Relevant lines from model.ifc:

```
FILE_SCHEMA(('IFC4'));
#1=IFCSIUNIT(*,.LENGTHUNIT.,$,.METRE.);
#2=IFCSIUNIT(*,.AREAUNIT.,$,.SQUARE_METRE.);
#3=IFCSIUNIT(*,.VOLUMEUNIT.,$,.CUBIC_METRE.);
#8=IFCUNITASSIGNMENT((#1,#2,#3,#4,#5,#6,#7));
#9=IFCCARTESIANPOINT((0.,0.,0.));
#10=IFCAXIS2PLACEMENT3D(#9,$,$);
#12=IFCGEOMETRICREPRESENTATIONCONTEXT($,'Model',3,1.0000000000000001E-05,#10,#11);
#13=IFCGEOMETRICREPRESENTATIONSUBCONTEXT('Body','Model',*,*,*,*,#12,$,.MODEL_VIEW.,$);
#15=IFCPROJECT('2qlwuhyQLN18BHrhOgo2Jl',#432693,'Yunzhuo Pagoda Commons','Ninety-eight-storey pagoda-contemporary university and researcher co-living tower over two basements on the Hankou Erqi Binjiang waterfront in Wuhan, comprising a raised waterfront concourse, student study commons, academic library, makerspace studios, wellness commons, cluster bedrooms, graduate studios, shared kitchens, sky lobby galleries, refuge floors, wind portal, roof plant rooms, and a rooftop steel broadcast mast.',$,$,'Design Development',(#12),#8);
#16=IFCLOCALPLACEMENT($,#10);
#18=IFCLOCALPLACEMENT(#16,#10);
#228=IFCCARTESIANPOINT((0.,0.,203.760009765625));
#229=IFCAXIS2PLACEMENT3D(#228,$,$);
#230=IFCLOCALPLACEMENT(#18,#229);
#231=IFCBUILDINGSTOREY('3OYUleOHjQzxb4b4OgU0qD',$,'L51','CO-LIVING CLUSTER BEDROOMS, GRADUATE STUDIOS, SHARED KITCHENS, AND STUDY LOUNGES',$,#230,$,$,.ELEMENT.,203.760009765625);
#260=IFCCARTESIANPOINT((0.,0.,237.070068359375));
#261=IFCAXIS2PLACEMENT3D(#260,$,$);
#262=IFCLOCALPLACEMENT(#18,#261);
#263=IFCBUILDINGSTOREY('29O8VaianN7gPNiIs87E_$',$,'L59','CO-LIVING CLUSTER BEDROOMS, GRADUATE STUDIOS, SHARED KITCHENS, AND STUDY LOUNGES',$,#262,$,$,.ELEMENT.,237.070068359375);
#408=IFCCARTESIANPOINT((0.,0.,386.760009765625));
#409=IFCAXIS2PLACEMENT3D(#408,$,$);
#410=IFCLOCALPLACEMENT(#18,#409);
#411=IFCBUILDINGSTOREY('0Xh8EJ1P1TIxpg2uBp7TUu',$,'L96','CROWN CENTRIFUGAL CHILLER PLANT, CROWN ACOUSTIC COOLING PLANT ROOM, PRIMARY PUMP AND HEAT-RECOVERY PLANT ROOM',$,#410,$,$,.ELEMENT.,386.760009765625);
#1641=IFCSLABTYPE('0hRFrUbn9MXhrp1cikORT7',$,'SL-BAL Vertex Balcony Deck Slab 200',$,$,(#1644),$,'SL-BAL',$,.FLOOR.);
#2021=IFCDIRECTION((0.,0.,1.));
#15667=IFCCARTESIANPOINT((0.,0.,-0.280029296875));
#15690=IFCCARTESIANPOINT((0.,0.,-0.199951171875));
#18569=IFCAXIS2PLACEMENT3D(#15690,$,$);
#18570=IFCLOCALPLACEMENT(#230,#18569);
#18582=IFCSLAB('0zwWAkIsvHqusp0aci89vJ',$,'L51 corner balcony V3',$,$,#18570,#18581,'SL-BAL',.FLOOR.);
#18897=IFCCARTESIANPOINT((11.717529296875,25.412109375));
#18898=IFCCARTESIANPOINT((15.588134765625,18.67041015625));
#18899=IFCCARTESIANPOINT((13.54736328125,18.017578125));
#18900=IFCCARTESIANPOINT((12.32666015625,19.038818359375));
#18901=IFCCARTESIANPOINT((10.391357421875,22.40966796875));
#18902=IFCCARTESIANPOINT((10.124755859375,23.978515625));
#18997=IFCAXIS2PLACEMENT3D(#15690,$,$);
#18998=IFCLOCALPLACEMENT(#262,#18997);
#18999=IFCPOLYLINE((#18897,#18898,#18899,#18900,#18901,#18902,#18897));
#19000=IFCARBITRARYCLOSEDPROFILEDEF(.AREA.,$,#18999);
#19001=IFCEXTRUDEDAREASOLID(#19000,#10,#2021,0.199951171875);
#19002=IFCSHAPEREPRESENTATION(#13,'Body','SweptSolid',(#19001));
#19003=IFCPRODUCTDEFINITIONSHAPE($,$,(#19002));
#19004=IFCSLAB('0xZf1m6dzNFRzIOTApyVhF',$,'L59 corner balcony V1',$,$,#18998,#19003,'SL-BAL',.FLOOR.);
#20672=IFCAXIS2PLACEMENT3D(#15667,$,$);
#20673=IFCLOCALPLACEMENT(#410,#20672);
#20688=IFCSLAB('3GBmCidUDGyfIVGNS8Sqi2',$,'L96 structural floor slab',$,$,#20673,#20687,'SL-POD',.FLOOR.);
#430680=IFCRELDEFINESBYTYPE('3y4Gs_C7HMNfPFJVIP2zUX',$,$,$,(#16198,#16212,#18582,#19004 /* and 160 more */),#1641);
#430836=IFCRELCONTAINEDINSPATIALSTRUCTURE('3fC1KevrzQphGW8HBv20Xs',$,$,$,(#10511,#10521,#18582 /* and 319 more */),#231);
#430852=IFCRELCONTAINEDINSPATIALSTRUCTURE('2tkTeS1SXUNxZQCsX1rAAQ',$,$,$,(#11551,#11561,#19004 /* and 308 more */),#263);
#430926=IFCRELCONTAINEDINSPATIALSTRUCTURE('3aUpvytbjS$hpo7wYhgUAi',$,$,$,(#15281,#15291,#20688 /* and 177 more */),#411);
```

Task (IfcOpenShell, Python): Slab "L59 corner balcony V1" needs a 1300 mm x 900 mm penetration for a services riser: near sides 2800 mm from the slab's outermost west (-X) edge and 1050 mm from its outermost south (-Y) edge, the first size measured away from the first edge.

```python
import numpy as np
import ifcopenshell
import ifcopenshell.api.feature
import ifcopenshell.api.geometry
import ifcopenshell.api.root
import ifcopenshell.geom
import ifcopenshell.util.placement
import ifcopenshell.util.representation
import ifcopenshell.util.shape
import ifcopenshell.util.unit

model = ifcopenshell.open("model.ifc")
unit_scale = ifcopenshell.util.unit.calculate_unit_scale(model)
settings = ifcopenshell.geom.settings()


def volume(element):
    """Net volume in cubic metres, openings subtracted."""
    shape = ifcopenshell.geom.create_shape(settings, element)
    return ifcopenshell.util.shape.get_volume(shape.geometry)


slab = model.by_guid("0xZf1m6dzNFRzIOTApyVhF")
before = volume(slab)

# Extent in the slab's own axes, in metres. The edges named are its -X and -Y sides.
slab_shape = ifcopenshell.geom.create_shape(settings, slab)
vertices = ifcopenshell.util.shape.get_vertices(slab_shape.geometry)
x_min, y_min, bottom = vertices.min(axis=0)
top = vertices[:, 2].max()

opening = ifcopenshell.api.root.create_entity(model, ifc_class="IfcOpeningElement", name="Services riser opening", predefined_type="OPENING")
context = ifcopenshell.util.representation.get_context(model, "Model", "Body", "MODEL_VIEW")
width, depth = 1.3, 0.9
outline = [(0.0, 0.0), (width, 0.0), (width, depth), (0.0, depth), (0.0, 0.0)]
# Overshoot both faces by 50 mm so the cut is clean.
shape = ifcopenshell.api.geometry.add_slab_representation(
    model, context=context, depth=top - bottom + 0.1, polyline=outline
)
ifcopenshell.api.geometry.assign_representation(model, product=opening, representation=shape)

matrix = ifcopenshell.util.placement.get_local_placement(slab.ObjectPlacement)
matrix[:, 3] = matrix @ np.append(np.array([x_min + 2.8, y_min + 1.05, bottom - 0.05]) / unit_scale, 1.0)
ifcopenshell.api.geometry.edit_object_placement(model, product=opening, matrix=matrix, is_si=False)
ifcopenshell.api.feature.add_feature(model, feature=opening, element=slab)

after = volume(slab)

print(f"slab volume {before:.3f} -> {after:.3f} m3")

model.write("model_rev.ifc")
```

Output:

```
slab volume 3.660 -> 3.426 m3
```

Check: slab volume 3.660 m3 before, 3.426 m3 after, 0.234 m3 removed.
